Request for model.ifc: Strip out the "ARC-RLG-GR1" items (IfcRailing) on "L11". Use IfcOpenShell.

First a look at what the model holds.

```python
import ifcopenshell
import ifcopenshell.util.element

model = ifcopenshell.open("model.ifc")
print(model.schema)
storey = next(s for s in model.by_type("IfcBuildingStorey") if s.Name == "L11")
railings = [e for e in ifcopenshell.util.element.get_decomposition(storey) if e.is_a("IfcRailing")]
seen = {}
for e in railings:
    element_type = ifcopenshell.util.element.get_type(e)
    name = element_type.Name if element_type not in (None, e) else None
    seen[name] = seen.get(name, 0) + 1
for name, count in sorted(seen.items(), key=str):
    print(count, "x", name)
```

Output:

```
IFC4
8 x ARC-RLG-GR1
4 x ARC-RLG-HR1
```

```python
import ifcopenshell
import ifcopenshell.api.root
import ifcopenshell.util.element

model = ifcopenshell.open("model.ifc")

storey = next(s for s in model.by_type("IfcBuildingStorey") if s.Name == "L11")
railings = [e for e in ifcopenshell.util.element.get_decomposition(storey) if e.is_a("IfcRailing")]
targets = [e for e in railings if (t := ifcopenshell.util.element.get_type(e)) not in (None, e) and t.Name == "ARC-RLG-GR1"]

for e in targets:
    ifcopenshell.api.root.remove_product(model, product=e)
print(len(targets), "removed")

model.write("model-out.ifc")
```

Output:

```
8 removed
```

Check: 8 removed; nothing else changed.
